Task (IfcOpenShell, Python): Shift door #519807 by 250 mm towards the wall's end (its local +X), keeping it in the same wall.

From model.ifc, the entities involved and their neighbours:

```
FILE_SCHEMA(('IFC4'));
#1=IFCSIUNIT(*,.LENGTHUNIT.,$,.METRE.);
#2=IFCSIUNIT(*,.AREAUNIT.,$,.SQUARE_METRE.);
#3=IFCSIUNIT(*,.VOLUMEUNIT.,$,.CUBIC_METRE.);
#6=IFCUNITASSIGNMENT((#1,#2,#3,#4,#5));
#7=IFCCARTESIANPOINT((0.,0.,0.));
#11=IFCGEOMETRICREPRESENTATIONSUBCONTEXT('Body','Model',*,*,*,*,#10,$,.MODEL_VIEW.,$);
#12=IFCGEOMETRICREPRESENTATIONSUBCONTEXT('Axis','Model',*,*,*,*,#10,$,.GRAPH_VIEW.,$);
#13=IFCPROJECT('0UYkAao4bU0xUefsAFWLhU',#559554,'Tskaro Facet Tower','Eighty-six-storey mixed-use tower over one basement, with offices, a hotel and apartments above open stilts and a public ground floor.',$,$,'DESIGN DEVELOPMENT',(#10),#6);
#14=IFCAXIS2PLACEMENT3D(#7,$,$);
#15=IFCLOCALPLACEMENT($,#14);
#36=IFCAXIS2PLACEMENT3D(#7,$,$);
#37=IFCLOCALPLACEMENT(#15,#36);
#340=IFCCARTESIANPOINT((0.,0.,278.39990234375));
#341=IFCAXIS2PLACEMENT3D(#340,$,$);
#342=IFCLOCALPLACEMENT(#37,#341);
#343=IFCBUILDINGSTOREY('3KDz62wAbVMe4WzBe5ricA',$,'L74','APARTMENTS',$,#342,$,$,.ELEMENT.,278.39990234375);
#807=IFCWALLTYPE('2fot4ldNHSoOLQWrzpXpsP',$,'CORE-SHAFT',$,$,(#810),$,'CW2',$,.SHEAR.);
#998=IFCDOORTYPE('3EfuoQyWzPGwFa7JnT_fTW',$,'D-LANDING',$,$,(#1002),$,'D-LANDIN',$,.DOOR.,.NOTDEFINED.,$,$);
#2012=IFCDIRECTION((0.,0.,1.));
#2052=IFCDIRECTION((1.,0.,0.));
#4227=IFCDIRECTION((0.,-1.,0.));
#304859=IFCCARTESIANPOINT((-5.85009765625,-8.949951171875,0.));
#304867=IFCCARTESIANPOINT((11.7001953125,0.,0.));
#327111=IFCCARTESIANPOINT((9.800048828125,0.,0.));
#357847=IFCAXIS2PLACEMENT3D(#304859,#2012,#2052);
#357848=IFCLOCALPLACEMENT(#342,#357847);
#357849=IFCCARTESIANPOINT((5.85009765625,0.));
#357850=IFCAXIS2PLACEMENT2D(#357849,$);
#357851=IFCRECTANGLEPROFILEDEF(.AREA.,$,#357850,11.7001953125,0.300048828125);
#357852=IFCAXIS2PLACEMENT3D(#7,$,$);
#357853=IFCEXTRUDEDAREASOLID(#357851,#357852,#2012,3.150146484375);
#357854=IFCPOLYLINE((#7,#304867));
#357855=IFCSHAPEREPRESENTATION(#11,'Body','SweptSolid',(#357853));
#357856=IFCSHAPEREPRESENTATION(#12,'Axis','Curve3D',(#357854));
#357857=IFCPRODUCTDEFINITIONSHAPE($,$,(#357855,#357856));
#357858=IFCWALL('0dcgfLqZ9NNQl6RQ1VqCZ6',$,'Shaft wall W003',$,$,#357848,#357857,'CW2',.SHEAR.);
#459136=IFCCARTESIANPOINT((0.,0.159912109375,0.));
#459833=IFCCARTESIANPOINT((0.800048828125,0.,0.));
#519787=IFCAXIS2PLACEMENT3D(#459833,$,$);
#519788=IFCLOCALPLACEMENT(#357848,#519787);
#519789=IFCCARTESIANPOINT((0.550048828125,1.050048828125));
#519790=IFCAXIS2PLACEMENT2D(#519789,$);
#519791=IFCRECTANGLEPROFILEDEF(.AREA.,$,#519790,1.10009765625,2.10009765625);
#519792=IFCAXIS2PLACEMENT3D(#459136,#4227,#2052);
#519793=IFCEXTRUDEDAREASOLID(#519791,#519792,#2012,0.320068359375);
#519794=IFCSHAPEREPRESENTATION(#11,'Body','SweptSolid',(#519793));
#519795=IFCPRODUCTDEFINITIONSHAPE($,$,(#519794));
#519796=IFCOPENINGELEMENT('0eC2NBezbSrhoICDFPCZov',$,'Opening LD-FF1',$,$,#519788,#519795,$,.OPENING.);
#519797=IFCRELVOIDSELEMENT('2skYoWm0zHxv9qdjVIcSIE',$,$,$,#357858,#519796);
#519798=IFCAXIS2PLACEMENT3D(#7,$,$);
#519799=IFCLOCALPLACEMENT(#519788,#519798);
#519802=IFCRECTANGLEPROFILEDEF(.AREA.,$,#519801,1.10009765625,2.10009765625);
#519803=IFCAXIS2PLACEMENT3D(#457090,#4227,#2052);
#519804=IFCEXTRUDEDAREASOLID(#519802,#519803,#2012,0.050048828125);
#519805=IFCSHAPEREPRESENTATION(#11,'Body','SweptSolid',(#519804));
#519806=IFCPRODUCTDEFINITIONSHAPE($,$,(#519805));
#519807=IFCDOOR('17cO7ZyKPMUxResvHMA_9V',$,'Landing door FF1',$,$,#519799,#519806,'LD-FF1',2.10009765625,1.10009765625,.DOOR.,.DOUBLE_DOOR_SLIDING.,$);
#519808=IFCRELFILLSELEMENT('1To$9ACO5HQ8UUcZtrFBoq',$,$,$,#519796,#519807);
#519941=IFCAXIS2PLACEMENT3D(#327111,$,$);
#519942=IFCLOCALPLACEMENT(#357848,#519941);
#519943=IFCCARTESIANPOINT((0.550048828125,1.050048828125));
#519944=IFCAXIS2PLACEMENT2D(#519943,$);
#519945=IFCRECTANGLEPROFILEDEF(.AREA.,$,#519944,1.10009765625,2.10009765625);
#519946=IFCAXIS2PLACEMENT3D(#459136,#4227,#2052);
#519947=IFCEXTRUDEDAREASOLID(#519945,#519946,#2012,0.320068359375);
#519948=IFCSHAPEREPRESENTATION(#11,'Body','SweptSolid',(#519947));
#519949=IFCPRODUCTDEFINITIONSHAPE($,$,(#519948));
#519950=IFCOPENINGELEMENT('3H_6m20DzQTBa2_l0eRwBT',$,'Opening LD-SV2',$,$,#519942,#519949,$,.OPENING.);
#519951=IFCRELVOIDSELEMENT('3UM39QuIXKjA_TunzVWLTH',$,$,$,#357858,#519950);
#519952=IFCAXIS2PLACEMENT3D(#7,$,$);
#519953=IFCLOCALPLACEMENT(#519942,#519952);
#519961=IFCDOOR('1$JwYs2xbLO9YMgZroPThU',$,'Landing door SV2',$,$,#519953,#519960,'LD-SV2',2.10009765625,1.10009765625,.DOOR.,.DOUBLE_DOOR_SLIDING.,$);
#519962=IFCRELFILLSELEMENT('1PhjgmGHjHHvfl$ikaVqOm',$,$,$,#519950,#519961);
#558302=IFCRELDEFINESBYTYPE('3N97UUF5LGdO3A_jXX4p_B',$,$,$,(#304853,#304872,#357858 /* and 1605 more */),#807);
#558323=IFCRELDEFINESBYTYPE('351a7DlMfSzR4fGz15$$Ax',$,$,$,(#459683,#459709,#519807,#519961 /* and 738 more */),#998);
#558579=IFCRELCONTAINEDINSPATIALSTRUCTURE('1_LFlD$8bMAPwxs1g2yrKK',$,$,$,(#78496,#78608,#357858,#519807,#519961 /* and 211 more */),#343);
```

```python
import ifcopenshell
import ifcopenshell.api.geometry
import ifcopenshell.util.placement
import ifcopenshell.util.unit

model = ifcopenshell.open("model.ifc")
unit_scale = ifcopenshell.util.unit.calculate_unit_scale(model)

door = model.by_guid("17cO7ZyKPMUxResvHMA_9V")
opening = door.FillsVoids[0].RelatingOpeningElement
wall = opening.VoidsElements[0].RelatingBuildingElement

wall_matrix = ifcopenshell.util.placement.get_local_placement(wall.ObjectPlacement)
shift = wall_matrix[:3, 0] * 0.25 / unit_scale
before = ifcopenshell.util.placement.get_local_placement(door.ObjectPlacement)[:3, 3].copy()

# The door is placed relative to its opening, so it follows when the opening moves.
matrix = ifcopenshell.util.placement.get_local_placement(opening.ObjectPlacement)
matrix[:3, 3] += shift
ifcopenshell.api.geometry.edit_object_placement(
    model, product=opening, matrix=matrix, is_si=False, should_transform_children=True
)

after = ifcopenshell.util.placement.get_local_placement(door.ObjectPlacement)[:3, 3]
print("door moved by", (after - before).round(3) + 0.0)

model.write("model_rev.ifc")
```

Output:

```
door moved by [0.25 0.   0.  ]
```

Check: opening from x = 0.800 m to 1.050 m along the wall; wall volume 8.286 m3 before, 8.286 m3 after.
